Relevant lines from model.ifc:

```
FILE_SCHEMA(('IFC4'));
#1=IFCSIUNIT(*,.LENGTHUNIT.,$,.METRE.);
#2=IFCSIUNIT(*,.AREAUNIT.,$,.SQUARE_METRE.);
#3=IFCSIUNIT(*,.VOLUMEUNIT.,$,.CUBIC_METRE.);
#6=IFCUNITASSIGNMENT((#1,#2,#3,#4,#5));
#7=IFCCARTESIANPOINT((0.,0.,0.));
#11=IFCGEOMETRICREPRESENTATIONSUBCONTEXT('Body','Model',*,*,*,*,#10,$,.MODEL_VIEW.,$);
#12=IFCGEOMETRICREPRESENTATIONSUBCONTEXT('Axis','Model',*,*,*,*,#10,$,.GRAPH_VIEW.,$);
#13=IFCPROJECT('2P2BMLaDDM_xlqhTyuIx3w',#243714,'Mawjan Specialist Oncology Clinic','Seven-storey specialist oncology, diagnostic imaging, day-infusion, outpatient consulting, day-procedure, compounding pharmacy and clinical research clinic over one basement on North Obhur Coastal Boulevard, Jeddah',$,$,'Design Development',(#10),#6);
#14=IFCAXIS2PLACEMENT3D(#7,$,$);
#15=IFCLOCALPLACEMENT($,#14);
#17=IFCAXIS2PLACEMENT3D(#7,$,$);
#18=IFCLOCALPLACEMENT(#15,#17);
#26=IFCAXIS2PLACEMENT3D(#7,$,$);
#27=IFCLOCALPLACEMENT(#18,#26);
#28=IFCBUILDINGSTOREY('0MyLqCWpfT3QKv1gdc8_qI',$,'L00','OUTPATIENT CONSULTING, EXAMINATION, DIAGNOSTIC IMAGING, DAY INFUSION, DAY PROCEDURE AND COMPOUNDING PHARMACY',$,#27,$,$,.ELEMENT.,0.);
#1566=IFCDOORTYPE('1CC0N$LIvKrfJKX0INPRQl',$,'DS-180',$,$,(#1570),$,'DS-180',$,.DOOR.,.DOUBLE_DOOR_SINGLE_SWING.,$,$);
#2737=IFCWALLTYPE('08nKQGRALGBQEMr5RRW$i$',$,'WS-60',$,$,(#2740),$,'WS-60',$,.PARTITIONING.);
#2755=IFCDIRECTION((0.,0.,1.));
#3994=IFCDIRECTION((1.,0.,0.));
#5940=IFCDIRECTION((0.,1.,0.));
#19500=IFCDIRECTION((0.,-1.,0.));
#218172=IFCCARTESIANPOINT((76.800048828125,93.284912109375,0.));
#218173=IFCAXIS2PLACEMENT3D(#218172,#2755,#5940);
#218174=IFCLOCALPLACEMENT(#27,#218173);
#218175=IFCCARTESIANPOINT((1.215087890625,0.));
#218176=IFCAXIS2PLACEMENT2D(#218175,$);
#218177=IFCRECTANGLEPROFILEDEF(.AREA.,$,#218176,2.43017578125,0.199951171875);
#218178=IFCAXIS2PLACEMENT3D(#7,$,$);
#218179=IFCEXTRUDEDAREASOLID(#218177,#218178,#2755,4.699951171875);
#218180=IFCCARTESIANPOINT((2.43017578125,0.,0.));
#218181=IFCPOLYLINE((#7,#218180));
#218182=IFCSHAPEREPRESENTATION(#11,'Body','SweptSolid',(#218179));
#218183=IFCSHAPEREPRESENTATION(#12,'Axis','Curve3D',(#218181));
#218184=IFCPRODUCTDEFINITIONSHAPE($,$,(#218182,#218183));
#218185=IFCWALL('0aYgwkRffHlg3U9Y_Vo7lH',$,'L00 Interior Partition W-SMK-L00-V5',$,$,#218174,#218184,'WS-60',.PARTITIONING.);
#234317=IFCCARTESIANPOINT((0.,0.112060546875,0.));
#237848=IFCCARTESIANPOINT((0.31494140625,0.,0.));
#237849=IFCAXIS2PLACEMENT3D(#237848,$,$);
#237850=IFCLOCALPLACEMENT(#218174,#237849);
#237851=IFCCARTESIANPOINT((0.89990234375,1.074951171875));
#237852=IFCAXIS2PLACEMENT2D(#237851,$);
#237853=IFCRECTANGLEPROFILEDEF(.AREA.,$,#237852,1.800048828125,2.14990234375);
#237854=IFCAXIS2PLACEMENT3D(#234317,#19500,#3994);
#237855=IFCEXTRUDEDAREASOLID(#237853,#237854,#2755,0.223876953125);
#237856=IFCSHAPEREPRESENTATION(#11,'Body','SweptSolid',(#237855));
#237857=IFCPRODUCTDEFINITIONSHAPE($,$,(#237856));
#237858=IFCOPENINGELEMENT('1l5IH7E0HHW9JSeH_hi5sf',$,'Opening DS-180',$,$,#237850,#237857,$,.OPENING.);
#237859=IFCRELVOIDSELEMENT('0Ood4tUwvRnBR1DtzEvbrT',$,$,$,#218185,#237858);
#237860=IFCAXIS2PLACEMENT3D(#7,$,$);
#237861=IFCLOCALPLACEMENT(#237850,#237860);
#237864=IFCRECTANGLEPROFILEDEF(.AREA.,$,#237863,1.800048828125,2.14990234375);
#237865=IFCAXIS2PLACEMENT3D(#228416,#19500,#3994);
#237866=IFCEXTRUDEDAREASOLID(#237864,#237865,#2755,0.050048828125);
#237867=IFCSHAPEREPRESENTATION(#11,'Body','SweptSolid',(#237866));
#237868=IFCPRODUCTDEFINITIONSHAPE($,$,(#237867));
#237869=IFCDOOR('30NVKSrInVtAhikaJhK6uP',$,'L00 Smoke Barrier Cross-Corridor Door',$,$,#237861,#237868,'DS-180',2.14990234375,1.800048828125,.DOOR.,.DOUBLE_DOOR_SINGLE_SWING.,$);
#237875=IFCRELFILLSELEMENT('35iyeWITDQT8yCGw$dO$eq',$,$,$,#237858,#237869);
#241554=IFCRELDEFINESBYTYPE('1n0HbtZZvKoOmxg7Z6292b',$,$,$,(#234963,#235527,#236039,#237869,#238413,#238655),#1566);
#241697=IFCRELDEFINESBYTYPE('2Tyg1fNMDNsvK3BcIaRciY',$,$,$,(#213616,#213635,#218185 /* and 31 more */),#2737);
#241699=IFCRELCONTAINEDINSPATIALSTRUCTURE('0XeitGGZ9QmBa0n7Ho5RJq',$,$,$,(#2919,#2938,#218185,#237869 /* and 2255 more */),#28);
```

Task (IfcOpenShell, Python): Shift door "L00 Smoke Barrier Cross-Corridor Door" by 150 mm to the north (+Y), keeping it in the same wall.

```python
import ifcopenshell
import ifcopenshell.api.geometry
import ifcopenshell.util.placement

model = ifcopenshell.open("model.ifc")

door = model.by_guid("30NVKSrInVtAhikaJhK6uP")
opening = door.FillsVoids[0].RelatingOpeningElement
wall = opening.VoidsElements[0].RelatingBuildingElement

wall_matrix = ifcopenshell.util.placement.get_local_placement(wall.ObjectPlacement)
shift = wall_matrix[:3, 0] * 0.15
before = ifcopenshell.util.placement.get_local_placement(door.ObjectPlacement)[:3, 3].copy()

# The door is placed relative to its opening, so it follows when the opening moves.
matrix = ifcopenshell.util.placement.get_local_placement(opening.ObjectPlacement)
matrix[:3, 3] += shift
ifcopenshell.api.geometry.edit_object_placement(
    model, product=opening, matrix=matrix, is_si=False, should_transform_children=True
)

after = ifcopenshell.util.placement.get_local_placement(door.ObjectPlacement)[:3, 3]
print("door moved by", (after - before).round(3) + 0.0)

model.write("model_rev.ifc")
```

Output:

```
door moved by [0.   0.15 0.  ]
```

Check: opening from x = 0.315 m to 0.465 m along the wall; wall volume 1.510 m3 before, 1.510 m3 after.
